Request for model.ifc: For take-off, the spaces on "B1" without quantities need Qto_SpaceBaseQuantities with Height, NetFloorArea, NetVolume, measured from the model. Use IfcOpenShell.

First a look at what the model holds.

```python
import ifcopenshell
import ifcopenshell.util.element
import ifcopenshell.util.unit

model = ifcopenshell.open("model.ifc")
print(model.schema)
for unit_type in ("LENGTHUNIT", "AREAUNIT", "VOLUMEUNIT"):
    print(unit_type, ifcopenshell.util.unit.calculate_unit_scale(model, unit_type))
storey = next(s for s in model.by_type("IfcBuildingStorey") if s.Name == "B1")
spaces = [e for e in ifcopenshell.util.element.get_decomposition(storey) if e.is_a("IfcSpace")]
for e in sorted(spaces, key=lambda e: e.id()):
    print(e.id(), e.is_a(), e.Name, list(ifcopenshell.util.element.get_psets(e, qtos_only=True)), sep=" | ")
```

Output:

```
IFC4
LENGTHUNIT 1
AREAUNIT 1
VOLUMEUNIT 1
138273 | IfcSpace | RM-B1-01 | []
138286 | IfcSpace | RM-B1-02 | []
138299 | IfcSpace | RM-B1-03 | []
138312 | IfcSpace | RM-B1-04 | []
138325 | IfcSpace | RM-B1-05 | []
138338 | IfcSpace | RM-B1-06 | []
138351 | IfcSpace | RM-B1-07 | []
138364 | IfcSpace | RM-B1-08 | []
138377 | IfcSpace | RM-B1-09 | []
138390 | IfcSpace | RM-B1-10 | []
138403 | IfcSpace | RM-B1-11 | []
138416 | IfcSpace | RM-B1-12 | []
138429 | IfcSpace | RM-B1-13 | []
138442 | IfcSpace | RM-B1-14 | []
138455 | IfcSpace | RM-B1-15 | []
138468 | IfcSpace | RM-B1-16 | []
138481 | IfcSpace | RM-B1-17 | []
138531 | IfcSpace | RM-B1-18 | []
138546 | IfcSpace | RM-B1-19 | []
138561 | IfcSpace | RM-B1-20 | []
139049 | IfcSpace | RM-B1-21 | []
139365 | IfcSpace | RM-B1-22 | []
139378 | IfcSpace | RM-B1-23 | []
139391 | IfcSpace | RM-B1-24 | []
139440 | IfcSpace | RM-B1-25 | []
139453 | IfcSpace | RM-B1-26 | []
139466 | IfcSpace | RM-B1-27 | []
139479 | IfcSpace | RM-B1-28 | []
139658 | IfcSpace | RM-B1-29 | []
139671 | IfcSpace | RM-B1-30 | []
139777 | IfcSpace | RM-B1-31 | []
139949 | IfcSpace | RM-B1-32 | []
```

```python
import ifcopenshell
import ifcopenshell.api.pset
import ifcopenshell.geom
import ifcopenshell.util.element
import ifcopenshell.util.shape
import ifcopenshell.util.unit

model = ifcopenshell.open("model.ifc")
unit_scale = ifcopenshell.util.unit.calculate_unit_scale(model)
area_scale = ifcopenshell.util.unit.calculate_unit_scale(model, "AREAUNIT")
volume_scale = ifcopenshell.util.unit.calculate_unit_scale(model, "VOLUMEUNIT")
settings = ifcopenshell.geom.settings()

storey = next(s for s in model.by_type("IfcBuildingStorey") if s.Name == "B1")
spaces = [e for e in ifcopenshell.util.element.get_decomposition(storey) if e.is_a("IfcSpace")]

for e in sorted(spaces, key=lambda e: e.id()):
    if ifcopenshell.util.element.get_psets(e, qtos_only=True, should_inherit=False):
        continue
    # Geometry comes back in metres, in the element's own axes.
    shape = ifcopenshell.geom.create_shape(settings, e)
    values = {
        "Height": ifcopenshell.util.shape.get_z(shape.geometry) / unit_scale,
        "NetFloorArea": ifcopenshell.util.shape.get_footprint_area(shape.geometry) / area_scale,
        "NetVolume": ifcopenshell.util.shape.get_volume(shape.geometry) / volume_scale,
    }
    qto = ifcopenshell.api.pset.add_qto(model, product=e, name="Qto_SpaceBaseQuantities")
    ifcopenshell.api.pset.edit_qto(model, qto=qto, properties=values)
    print(e.id(), {k: round(v, 3) for k, v in values.items()})

model.write("model_rev.ifc")
```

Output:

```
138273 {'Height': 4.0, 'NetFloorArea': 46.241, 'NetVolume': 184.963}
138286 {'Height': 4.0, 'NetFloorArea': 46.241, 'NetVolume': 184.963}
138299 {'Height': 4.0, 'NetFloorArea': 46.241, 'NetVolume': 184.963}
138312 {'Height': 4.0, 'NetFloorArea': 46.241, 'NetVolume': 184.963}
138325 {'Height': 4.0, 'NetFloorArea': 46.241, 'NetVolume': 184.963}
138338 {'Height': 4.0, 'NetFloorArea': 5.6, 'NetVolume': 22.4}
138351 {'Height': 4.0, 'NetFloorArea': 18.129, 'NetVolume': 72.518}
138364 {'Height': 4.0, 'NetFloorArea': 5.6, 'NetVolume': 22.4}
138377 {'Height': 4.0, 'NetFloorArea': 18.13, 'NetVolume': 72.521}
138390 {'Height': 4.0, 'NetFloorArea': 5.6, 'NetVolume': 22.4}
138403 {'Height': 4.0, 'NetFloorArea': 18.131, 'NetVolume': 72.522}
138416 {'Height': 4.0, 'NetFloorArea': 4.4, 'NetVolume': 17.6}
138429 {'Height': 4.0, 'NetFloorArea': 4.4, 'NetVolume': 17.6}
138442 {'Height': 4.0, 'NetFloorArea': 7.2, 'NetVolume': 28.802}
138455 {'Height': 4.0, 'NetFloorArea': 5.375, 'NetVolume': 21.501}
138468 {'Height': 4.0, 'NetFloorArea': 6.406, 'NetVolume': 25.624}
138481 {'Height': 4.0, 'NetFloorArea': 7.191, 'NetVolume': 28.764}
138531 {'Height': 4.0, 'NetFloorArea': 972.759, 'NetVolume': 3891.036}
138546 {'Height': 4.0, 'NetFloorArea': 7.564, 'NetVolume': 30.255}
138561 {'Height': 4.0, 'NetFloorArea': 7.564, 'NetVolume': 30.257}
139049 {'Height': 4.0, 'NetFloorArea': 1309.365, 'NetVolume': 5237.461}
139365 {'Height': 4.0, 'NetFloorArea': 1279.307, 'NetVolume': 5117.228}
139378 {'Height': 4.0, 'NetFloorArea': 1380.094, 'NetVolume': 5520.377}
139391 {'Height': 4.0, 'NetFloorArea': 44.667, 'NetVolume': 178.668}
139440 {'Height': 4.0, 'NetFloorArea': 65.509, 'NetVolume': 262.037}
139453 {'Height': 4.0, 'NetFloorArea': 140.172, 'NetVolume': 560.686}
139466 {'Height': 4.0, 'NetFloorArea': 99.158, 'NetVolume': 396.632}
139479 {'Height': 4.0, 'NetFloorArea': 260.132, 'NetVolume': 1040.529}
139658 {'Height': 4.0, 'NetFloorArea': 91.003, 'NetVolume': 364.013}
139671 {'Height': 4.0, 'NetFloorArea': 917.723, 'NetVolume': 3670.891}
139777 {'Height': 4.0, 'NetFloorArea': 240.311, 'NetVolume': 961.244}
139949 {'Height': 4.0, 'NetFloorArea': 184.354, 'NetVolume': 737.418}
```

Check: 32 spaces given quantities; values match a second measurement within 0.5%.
